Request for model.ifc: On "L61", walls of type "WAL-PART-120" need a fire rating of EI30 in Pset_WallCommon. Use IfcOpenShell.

First a look at what the model holds.

```python
import ifcopenshell
import ifcopenshell.util.element

model = ifcopenshell.open("model.ifc")
print(model.schema)
storey = next(s for s in model.by_type("IfcBuildingStorey") if s.Name == "L61")
walls = [e for e in ifcopenshell.util.element.get_decomposition(storey) if e.is_a("IfcWall")]
seen = {}
for e in walls:
    element_type = ifcopenshell.util.element.get_type(e)
    key = (element_type.Name if element_type != e and element_type else None, ifcopenshell.util.element.get_pset(e, "Pset_WallCommon", "FireRating"))
    seen[key] = seen.get(key, 0) + 1
for (name, value), count in sorted(seen.items(), key=str):
    print(count, "x", name, "|", value)
```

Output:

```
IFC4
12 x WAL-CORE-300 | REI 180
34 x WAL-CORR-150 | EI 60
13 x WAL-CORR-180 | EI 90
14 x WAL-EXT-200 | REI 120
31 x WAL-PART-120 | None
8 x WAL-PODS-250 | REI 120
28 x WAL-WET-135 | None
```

```python
import ifcopenshell
import ifcopenshell.api.pset
import ifcopenshell.util.element

model = ifcopenshell.open("model.ifc")

storey = next(s for s in model.by_type("IfcBuildingStorey") if s.Name == "L61")
walls = [e for e in ifcopenshell.util.element.get_decomposition(storey) if e.is_a("IfcWall")]

count = 0
for e in walls:
    element_type = ifcopenshell.util.element.get_type(e)
    if element_type in (None, e) or element_type.Name != "WAL-PART-120":
        continue
    # add_pset returns the element's existing set when there is one.
    pset = ifcopenshell.api.pset.add_pset(model, product=e, name="Pset_WallCommon")
    ifcopenshell.api.pset.edit_pset(model, pset=pset, properties={"FireRating": "EI30"})
    count += 1

print(count, "walls updated")

model.write("model_rev.ifc")
```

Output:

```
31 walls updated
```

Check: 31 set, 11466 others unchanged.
